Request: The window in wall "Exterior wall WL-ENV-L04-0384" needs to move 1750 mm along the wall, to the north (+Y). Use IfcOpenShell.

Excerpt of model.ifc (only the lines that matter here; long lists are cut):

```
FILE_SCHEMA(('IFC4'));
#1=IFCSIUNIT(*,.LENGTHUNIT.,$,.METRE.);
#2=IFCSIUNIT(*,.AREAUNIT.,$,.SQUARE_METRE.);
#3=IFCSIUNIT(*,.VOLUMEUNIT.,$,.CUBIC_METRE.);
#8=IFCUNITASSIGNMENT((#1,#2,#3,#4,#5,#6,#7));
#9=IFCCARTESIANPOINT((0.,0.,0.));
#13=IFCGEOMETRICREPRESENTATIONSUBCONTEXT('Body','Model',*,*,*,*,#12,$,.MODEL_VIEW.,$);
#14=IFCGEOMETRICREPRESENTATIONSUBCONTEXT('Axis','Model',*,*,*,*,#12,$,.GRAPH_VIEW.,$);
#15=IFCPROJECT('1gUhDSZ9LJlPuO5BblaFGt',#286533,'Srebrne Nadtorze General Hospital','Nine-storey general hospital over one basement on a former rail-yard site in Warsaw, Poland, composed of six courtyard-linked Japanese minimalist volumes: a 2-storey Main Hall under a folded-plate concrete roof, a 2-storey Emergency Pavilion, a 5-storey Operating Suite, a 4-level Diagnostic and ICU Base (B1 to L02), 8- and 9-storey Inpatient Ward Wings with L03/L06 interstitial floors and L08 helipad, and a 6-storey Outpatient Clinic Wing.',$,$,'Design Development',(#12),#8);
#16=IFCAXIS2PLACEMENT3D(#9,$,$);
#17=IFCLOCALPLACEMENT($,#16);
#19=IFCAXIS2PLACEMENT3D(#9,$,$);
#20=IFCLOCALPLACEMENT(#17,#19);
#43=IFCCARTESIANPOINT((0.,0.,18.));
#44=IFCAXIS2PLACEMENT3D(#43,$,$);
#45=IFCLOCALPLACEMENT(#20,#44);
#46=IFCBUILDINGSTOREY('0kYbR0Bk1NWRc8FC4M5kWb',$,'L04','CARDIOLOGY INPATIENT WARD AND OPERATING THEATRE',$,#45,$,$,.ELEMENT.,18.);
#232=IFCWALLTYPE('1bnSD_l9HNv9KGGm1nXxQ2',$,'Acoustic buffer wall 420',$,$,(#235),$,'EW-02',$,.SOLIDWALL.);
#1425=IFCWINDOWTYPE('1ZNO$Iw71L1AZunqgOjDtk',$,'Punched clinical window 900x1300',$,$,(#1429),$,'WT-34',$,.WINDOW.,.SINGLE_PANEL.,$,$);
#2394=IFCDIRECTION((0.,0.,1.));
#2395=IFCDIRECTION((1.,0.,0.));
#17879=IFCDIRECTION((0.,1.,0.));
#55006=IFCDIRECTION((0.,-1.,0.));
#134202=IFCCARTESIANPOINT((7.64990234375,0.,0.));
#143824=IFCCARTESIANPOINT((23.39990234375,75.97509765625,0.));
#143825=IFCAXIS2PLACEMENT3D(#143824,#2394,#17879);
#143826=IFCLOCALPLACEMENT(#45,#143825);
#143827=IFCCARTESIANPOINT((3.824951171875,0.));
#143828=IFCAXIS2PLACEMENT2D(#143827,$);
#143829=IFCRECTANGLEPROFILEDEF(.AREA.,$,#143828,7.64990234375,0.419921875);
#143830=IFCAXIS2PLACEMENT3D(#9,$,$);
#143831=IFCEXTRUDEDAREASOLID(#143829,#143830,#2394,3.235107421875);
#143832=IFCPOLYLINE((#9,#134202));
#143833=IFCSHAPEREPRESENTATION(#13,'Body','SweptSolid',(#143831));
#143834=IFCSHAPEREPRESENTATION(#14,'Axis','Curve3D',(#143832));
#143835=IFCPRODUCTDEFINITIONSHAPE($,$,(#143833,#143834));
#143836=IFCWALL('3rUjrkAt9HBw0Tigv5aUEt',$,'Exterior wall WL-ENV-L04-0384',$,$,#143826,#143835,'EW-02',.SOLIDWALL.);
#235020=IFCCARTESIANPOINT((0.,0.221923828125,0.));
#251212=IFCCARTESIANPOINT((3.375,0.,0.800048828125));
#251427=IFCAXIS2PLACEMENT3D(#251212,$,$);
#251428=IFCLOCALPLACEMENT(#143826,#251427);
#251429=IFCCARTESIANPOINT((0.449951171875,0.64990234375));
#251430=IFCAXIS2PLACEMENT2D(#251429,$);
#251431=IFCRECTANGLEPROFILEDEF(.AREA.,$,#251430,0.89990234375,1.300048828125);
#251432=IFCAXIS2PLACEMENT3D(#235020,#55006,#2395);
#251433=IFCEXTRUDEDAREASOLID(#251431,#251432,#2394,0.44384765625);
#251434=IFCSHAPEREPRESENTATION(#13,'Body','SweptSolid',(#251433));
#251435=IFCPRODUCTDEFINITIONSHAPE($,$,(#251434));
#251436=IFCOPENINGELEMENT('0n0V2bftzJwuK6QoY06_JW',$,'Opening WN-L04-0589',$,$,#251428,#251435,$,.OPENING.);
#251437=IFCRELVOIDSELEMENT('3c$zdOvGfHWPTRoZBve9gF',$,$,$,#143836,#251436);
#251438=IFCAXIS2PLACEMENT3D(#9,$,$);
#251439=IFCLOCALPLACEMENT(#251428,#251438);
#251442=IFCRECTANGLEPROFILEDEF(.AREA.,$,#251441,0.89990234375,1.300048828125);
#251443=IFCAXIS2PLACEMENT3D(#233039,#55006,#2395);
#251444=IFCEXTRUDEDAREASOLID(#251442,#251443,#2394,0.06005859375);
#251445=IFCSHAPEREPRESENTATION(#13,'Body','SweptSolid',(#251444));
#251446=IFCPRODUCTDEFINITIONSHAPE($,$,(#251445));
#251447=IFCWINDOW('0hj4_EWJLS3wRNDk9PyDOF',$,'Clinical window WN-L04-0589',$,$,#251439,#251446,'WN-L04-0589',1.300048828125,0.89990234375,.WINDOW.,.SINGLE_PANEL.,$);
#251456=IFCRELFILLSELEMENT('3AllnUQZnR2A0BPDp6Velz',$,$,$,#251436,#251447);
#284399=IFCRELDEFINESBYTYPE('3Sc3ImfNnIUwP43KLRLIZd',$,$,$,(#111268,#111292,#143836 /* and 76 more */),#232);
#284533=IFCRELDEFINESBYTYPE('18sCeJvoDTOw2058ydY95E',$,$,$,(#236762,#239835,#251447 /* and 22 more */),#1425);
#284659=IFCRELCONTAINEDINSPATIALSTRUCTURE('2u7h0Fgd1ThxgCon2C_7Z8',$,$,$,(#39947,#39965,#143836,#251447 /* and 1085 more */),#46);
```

```python
import ifcopenshell
import ifcopenshell.api.geometry
import ifcopenshell.util.placement
import ifcopenshell.util.unit

model = ifcopenshell.open("model.ifc")
unit_scale = ifcopenshell.util.unit.calculate_unit_scale(model)

window = model.by_guid("0hj4_EWJLS3wRNDk9PyDOF")
opening = window.FillsVoids[0].RelatingOpeningElement
wall = opening.VoidsElements[0].RelatingBuildingElement

wall_matrix = ifcopenshell.util.placement.get_local_placement(wall.ObjectPlacement)
shift = wall_matrix[:3, 0] * 1.75 / unit_scale
before = ifcopenshell.util.placement.get_local_placement(window.ObjectPlacement)[:3, 3].copy()

# The window is placed relative to its opening, so it follows when the opening moves.
matrix = ifcopenshell.util.placement.get_local_placement(opening.ObjectPlacement)
matrix[:3, 3] += shift
ifcopenshell.api.geometry.edit_object_placement(
    model, product=opening, matrix=matrix, is_si=False, should_transform_children=True
)

after = ifcopenshell.util.placement.get_local_placement(window.ObjectPlacement)[:3, 3]
print("window moved by", (after - before).round(3) + 0.0)

model.write("model-out.ifc")
```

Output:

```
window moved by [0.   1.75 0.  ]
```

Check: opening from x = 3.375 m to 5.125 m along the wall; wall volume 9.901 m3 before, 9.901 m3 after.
